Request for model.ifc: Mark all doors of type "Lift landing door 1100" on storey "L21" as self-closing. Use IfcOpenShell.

First a look at what the model holds.

```python
import ifcopenshell
import ifcopenshell.util.element

model = ifcopenshell.open("model.ifc")
print(model.schema)
storey = next(s for s in model.by_type("IfcBuildingStorey") if s.Name == "L21")
doors = [e for e in ifcopenshell.util.element.get_decomposition(storey) if e.is_a("IfcDoor")]
seen = {}
for e in doors:
    element_type = ifcopenshell.util.element.get_type(e)
    key = (element_type.Name if element_type != e and element_type else None, ifcopenshell.util.element.get_pset(e, "Pset_DoorCommon", "SelfClosing"))
    seen[key] = seen.get(key, 0) + 1
for (name, value), count in sorted(seen.items(), key=str):
    print(count, "x", name, "|", value)
```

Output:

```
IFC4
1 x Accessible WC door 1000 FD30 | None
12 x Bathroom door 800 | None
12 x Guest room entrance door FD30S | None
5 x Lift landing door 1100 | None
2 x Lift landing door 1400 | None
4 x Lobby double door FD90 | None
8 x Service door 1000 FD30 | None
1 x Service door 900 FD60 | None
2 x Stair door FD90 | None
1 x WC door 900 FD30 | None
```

```python
import ifcopenshell
import ifcopenshell.api.pset
import ifcopenshell.util.element

model = ifcopenshell.open("model.ifc")

storey = next(s for s in model.by_type("IfcBuildingStorey") if s.Name == "L21")
doors = [e for e in ifcopenshell.util.element.get_decomposition(storey) if e.is_a("IfcDoor")]

count = 0
for e in doors:
    element_type = ifcopenshell.util.element.get_type(e)
    if element_type in (None, e) or element_type.Name != "Lift landing door 1100":
        continue
    # add_pset returns the element's existing set when there is one.
    pset = ifcopenshell.api.pset.add_pset(model, product=e, name="Pset_DoorCommon")
    ifcopenshell.api.pset.edit_pset(model, pset=pset, properties={"SelfClosing": True})
    count += 1

print(count, "doors updated")

model.write("model_updated.ifc")
```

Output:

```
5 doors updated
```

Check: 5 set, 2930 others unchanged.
